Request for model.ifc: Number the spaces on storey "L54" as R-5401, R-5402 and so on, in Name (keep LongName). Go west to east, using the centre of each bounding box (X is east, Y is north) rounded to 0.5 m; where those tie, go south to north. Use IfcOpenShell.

First a look at what the model holds.

```python
import ifcopenshell
import ifcopenshell.util.element
import ifcopenshell.util.placement

model = ifcopenshell.open("model.ifc")
print(model.schema)
storey = next(s for s in model.by_type("IfcBuildingStorey") if s.Name == "L54")
spaces = [e for e in ifcopenshell.util.element.get_decomposition(storey) if e.is_a("IfcSpace")]
for e in sorted(spaces, key=lambda e: e.id()):
    origin = ifcopenshell.util.placement.get_local_placement(e.ObjectPlacement)[:3, 3]
    print(e.id(), e.Name, e.LongName, origin.round(2) + 0.0, sep=" | ")
```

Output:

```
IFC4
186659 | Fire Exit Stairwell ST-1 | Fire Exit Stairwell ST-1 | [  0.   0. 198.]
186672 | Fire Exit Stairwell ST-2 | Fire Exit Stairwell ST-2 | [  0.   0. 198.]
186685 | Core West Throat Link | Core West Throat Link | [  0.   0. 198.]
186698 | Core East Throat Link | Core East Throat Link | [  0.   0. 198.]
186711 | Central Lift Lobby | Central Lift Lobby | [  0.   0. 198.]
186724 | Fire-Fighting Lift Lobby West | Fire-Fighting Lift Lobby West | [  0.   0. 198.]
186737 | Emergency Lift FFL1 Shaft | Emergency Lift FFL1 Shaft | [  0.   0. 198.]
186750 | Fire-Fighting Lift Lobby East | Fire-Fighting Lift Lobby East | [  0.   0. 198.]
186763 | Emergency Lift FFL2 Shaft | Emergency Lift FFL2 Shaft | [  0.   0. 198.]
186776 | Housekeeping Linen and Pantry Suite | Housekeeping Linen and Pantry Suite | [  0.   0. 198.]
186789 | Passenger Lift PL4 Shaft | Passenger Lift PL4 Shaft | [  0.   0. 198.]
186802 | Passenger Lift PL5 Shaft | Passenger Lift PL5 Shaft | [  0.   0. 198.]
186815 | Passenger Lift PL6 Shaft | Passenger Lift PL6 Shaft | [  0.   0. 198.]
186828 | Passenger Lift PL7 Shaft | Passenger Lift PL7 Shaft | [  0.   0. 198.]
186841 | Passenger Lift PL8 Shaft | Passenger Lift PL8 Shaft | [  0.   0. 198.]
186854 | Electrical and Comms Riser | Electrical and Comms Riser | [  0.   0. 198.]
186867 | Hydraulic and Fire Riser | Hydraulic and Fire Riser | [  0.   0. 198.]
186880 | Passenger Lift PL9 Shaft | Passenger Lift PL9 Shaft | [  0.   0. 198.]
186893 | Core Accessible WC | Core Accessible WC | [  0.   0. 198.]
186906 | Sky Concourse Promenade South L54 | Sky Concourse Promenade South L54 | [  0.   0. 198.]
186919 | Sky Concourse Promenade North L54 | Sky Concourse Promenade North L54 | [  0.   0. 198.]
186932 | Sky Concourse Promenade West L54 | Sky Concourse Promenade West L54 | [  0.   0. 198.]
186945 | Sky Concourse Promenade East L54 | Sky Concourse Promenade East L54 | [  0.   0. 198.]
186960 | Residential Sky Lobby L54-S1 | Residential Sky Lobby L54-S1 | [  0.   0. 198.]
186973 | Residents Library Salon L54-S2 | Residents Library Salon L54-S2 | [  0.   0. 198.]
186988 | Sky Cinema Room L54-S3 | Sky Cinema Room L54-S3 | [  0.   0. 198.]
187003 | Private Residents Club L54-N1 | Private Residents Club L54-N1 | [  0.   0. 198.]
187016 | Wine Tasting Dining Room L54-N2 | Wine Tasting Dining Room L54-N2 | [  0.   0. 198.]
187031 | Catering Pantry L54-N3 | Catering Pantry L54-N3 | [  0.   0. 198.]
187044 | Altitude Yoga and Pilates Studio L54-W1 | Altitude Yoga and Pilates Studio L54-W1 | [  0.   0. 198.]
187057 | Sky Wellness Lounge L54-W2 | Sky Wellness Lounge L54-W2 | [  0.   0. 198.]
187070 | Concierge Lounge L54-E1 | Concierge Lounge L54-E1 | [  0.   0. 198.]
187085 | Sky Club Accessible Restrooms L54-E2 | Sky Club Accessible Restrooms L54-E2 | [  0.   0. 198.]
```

```python
import ifcopenshell
import ifcopenshell.geom
import ifcopenshell.util.element
import ifcopenshell.util.shape

model = ifcopenshell.open("model.ifc")
settings = ifcopenshell.geom.settings()
settings.set("use-world-coords", True)


def centre(element):
    shape = ifcopenshell.geom.create_shape(settings, element)
    return ifcopenshell.util.shape.get_bbox_centroid(shape.geometry)


storey = next(s for s in model.by_type("IfcBuildingStorey") if s.Name == "L54")
spaces = [e for e in ifcopenshell.util.element.get_decomposition(storey) if e.is_a("IfcSpace")]

# Insertion points can sit at a corner or the storey origin, so sort by the geometry (in metres).
centres = {e: centre(e) for e in spaces}
spaces.sort(key=lambda e: (round(centres[e][0] / 0.5), centres[e][1]))

for i, e in enumerate(spaces, start=1):
    number = f"R-54{i:02d}"
    e.Name = number
    print(e.id(), number)

model.write("model_v2.ifc")
```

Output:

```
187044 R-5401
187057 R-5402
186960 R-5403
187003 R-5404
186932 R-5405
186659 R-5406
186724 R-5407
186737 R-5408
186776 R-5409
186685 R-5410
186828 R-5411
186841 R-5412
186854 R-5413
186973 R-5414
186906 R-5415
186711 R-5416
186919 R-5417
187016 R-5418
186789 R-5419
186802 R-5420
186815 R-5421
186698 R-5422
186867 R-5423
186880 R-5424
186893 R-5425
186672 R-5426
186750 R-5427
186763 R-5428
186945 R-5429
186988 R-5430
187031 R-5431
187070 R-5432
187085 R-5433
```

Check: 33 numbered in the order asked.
